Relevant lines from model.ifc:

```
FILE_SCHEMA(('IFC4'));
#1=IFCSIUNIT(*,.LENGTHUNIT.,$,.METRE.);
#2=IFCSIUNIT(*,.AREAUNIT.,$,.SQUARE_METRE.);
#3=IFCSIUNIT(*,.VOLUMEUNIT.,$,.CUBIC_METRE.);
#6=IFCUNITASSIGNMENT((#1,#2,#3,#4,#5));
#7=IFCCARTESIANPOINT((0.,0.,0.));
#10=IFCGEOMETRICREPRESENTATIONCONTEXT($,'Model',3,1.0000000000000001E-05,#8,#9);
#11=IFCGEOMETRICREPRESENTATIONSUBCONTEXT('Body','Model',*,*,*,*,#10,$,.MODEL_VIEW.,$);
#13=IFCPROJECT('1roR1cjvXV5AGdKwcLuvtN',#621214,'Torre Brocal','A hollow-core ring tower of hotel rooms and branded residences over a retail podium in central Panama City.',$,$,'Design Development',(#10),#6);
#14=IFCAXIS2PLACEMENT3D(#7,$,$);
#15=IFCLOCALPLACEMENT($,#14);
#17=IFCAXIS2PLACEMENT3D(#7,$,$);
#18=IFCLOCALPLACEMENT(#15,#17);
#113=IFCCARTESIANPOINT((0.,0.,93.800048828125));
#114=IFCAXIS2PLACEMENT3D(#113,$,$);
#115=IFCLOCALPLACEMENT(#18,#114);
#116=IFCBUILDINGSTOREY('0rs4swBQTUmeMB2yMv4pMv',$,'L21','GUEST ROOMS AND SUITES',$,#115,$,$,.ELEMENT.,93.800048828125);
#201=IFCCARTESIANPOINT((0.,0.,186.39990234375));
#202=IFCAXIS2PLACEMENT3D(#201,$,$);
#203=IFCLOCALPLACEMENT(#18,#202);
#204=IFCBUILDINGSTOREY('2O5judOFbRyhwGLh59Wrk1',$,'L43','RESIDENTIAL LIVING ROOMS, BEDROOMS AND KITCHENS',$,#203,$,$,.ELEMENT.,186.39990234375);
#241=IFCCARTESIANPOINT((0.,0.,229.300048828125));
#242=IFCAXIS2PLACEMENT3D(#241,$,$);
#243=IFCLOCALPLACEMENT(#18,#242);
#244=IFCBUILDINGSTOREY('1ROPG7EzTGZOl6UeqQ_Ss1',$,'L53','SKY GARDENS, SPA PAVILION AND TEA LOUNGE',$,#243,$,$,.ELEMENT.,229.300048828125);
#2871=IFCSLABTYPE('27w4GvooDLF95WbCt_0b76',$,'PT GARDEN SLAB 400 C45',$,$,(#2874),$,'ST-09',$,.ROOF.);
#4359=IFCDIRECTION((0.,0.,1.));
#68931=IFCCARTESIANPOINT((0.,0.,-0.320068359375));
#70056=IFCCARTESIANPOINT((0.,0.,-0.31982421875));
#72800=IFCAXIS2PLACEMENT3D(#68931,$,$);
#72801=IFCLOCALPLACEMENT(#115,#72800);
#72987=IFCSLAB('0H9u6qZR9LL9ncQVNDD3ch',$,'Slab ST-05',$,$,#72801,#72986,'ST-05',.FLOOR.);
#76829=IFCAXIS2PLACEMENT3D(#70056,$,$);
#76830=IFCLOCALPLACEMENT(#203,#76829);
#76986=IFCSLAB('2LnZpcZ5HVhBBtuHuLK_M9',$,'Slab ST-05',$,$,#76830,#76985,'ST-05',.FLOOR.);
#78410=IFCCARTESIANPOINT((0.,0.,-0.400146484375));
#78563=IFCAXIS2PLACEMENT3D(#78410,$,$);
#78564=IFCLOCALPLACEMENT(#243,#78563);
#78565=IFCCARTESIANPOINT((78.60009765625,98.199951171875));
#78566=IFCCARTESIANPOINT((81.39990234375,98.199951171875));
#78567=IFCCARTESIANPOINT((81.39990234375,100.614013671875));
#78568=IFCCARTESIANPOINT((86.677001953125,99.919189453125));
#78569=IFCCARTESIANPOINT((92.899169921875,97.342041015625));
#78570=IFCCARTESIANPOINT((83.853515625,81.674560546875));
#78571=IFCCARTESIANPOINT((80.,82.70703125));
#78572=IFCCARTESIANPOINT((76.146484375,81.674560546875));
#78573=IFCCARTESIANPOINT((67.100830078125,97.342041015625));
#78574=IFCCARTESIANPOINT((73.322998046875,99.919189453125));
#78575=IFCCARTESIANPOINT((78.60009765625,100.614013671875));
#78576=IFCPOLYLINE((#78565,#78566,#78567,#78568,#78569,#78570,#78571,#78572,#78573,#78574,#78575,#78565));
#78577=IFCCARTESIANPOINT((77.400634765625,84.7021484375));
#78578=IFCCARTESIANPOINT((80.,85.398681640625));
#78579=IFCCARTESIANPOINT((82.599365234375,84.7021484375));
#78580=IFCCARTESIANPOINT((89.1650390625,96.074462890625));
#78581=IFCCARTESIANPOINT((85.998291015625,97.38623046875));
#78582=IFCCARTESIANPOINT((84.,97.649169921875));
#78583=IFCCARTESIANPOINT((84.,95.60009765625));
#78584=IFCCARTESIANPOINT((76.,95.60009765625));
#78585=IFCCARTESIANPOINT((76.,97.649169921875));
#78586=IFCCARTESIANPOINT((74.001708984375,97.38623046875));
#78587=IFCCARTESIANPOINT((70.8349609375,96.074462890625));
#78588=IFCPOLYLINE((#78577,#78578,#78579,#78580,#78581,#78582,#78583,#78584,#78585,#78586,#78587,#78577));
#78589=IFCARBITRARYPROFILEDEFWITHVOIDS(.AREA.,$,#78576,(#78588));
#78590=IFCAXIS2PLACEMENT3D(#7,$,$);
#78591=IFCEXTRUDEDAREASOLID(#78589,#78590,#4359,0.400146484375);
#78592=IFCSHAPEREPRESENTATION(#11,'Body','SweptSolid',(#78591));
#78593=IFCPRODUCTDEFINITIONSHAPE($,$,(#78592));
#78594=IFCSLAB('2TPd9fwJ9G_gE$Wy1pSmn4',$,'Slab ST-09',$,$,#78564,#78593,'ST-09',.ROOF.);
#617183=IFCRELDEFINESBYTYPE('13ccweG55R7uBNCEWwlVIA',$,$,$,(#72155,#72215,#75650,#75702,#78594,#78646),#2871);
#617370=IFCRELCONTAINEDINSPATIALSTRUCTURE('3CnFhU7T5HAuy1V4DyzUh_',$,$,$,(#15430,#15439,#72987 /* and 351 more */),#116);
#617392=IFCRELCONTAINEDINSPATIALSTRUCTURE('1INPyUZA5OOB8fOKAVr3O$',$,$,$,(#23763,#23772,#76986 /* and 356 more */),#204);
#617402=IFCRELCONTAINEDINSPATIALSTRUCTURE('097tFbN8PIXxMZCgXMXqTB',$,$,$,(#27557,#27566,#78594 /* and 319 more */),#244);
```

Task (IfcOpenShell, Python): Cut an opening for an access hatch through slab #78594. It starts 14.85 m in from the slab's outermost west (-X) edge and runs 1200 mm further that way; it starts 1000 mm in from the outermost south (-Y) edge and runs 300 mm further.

```python
import numpy as np
import ifcopenshell
import ifcopenshell.api.feature
import ifcopenshell.api.geometry
import ifcopenshell.api.root
import ifcopenshell.geom
import ifcopenshell.util.placement
import ifcopenshell.util.representation
import ifcopenshell.util.shape
import ifcopenshell.util.unit

model = ifcopenshell.open("model.ifc")
unit_scale = ifcopenshell.util.unit.calculate_unit_scale(model)
settings = ifcopenshell.geom.settings()


def volume(element):
    """Net volume in cubic metres, openings subtracted."""
    shape = ifcopenshell.geom.create_shape(settings, element)
    return ifcopenshell.util.shape.get_volume(shape.geometry)


slab = model.by_id(78594)
before = volume(slab)

# Extent in the slab's own axes, in metres. The edges named are its -X and -Y sides.
slab_shape = ifcopenshell.geom.create_shape(settings, slab)
vertices = ifcopenshell.util.shape.get_vertices(slab_shape.geometry)
x_min, y_min, bottom = vertices.min(axis=0)
top = vertices[:, 2].max()

opening = ifcopenshell.api.root.create_entity(model, ifc_class="IfcOpeningElement", name="Access hatch opening", predefined_type="OPENING")
context = ifcopenshell.util.representation.get_context(model, "Model", "Body", "MODEL_VIEW")
width, depth = 1.2, 0.3
outline = [(0.0, 0.0), (width, 0.0), (width, depth), (0.0, depth), (0.0, 0.0)]
# Overshoot both faces by 50 mm so the cut is clean.
shape = ifcopenshell.api.geometry.add_slab_representation(
    model, context=context, depth=top - bottom + 0.1, polyline=outline
)
ifcopenshell.api.geometry.assign_representation(model, product=opening, representation=shape)

matrix = ifcopenshell.util.placement.get_local_placement(slab.ObjectPlacement)
matrix[:, 3] = matrix @ np.append(np.array([x_min + 14.85, y_min + 1, bottom - 0.05]) / unit_scale, 1.0)
ifcopenshell.api.geometry.edit_object_placement(model, product=opening, matrix=matrix, is_si=False)
ifcopenshell.api.feature.add_feature(model, feature=opening, element=slab)

after = volume(slab)

print(f"slab volume {before:.3f} -> {after:.3f} m3")

model.write("model-out.ifc")
```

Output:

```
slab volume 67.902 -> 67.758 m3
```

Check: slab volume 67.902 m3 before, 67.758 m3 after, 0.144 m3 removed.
